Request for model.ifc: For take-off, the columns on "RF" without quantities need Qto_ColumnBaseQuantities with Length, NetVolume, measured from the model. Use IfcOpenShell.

First a look at what the model holds.

```python
import ifcopenshell
import ifcopenshell.util.element
import ifcopenshell.util.unit

model = ifcopenshell.open("model.ifc")
print(model.schema)
for unit_type in ("LENGTHUNIT", "AREAUNIT", "VOLUMEUNIT"):
    print(unit_type, ifcopenshell.util.unit.calculate_unit_scale(model, unit_type))
storey = next(s for s in model.by_type("IfcBuildingStorey") if s.Name == "RF")
columns = [e for e in ifcopenshell.util.element.get_decomposition(storey) if e.is_a("IfcColumn")]
for e in sorted(columns, key=lambda e: e.id()):
    print(e.id(), e.is_a(), e.Name, list(ifcopenshell.util.element.get_psets(e, qtos_only=True)), sep=" | ")
```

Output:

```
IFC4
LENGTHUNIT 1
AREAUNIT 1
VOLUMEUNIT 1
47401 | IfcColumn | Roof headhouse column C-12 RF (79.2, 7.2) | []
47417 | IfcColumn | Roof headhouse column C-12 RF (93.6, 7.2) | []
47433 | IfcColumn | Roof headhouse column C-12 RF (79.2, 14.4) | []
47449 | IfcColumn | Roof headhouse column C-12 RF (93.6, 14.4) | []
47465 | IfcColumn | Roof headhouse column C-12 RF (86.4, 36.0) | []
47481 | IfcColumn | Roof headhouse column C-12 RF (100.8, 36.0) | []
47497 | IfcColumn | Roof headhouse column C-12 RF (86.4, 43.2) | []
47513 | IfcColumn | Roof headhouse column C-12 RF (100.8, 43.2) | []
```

```python
import ifcopenshell
import ifcopenshell.api.pset
import ifcopenshell.geom
import ifcopenshell.util.element
import ifcopenshell.util.shape
import ifcopenshell.util.unit

model = ifcopenshell.open("model.ifc")
unit_scale = ifcopenshell.util.unit.calculate_unit_scale(model)
volume_scale = ifcopenshell.util.unit.calculate_unit_scale(model, "VOLUMEUNIT")
settings = ifcopenshell.geom.settings()

storey = next(s for s in model.by_type("IfcBuildingStorey") if s.Name == "RF")
columns = [e for e in ifcopenshell.util.element.get_decomposition(storey) if e.is_a("IfcColumn")]

for e in sorted(columns, key=lambda e: e.id()):
    if ifcopenshell.util.element.get_psets(e, qtos_only=True, should_inherit=False):
        continue
    # Geometry comes back in metres, in the element's own axes.
    shape = ifcopenshell.geom.create_shape(settings, e)
    values = {
        "Length": ifcopenshell.util.shape.get_z(shape.geometry) / unit_scale,
        "NetVolume": ifcopenshell.util.shape.get_volume(shape.geometry) / volume_scale,
    }
    qto = ifcopenshell.api.pset.add_qto(model, product=e, name="Qto_ColumnBaseQuantities")
    ifcopenshell.api.pset.edit_qto(model, qto=qto, properties=values)
    print(e.id(), {k: round(v, 3) for k, v in values.items()})

model.write("model_rev.ifc")
```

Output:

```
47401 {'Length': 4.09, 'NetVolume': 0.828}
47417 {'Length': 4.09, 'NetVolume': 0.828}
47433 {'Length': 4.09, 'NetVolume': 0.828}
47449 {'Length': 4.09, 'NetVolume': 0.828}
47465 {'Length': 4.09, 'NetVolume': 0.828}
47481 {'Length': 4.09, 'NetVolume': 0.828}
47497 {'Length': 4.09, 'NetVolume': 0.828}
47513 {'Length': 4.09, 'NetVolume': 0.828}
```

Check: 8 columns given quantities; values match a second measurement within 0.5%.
